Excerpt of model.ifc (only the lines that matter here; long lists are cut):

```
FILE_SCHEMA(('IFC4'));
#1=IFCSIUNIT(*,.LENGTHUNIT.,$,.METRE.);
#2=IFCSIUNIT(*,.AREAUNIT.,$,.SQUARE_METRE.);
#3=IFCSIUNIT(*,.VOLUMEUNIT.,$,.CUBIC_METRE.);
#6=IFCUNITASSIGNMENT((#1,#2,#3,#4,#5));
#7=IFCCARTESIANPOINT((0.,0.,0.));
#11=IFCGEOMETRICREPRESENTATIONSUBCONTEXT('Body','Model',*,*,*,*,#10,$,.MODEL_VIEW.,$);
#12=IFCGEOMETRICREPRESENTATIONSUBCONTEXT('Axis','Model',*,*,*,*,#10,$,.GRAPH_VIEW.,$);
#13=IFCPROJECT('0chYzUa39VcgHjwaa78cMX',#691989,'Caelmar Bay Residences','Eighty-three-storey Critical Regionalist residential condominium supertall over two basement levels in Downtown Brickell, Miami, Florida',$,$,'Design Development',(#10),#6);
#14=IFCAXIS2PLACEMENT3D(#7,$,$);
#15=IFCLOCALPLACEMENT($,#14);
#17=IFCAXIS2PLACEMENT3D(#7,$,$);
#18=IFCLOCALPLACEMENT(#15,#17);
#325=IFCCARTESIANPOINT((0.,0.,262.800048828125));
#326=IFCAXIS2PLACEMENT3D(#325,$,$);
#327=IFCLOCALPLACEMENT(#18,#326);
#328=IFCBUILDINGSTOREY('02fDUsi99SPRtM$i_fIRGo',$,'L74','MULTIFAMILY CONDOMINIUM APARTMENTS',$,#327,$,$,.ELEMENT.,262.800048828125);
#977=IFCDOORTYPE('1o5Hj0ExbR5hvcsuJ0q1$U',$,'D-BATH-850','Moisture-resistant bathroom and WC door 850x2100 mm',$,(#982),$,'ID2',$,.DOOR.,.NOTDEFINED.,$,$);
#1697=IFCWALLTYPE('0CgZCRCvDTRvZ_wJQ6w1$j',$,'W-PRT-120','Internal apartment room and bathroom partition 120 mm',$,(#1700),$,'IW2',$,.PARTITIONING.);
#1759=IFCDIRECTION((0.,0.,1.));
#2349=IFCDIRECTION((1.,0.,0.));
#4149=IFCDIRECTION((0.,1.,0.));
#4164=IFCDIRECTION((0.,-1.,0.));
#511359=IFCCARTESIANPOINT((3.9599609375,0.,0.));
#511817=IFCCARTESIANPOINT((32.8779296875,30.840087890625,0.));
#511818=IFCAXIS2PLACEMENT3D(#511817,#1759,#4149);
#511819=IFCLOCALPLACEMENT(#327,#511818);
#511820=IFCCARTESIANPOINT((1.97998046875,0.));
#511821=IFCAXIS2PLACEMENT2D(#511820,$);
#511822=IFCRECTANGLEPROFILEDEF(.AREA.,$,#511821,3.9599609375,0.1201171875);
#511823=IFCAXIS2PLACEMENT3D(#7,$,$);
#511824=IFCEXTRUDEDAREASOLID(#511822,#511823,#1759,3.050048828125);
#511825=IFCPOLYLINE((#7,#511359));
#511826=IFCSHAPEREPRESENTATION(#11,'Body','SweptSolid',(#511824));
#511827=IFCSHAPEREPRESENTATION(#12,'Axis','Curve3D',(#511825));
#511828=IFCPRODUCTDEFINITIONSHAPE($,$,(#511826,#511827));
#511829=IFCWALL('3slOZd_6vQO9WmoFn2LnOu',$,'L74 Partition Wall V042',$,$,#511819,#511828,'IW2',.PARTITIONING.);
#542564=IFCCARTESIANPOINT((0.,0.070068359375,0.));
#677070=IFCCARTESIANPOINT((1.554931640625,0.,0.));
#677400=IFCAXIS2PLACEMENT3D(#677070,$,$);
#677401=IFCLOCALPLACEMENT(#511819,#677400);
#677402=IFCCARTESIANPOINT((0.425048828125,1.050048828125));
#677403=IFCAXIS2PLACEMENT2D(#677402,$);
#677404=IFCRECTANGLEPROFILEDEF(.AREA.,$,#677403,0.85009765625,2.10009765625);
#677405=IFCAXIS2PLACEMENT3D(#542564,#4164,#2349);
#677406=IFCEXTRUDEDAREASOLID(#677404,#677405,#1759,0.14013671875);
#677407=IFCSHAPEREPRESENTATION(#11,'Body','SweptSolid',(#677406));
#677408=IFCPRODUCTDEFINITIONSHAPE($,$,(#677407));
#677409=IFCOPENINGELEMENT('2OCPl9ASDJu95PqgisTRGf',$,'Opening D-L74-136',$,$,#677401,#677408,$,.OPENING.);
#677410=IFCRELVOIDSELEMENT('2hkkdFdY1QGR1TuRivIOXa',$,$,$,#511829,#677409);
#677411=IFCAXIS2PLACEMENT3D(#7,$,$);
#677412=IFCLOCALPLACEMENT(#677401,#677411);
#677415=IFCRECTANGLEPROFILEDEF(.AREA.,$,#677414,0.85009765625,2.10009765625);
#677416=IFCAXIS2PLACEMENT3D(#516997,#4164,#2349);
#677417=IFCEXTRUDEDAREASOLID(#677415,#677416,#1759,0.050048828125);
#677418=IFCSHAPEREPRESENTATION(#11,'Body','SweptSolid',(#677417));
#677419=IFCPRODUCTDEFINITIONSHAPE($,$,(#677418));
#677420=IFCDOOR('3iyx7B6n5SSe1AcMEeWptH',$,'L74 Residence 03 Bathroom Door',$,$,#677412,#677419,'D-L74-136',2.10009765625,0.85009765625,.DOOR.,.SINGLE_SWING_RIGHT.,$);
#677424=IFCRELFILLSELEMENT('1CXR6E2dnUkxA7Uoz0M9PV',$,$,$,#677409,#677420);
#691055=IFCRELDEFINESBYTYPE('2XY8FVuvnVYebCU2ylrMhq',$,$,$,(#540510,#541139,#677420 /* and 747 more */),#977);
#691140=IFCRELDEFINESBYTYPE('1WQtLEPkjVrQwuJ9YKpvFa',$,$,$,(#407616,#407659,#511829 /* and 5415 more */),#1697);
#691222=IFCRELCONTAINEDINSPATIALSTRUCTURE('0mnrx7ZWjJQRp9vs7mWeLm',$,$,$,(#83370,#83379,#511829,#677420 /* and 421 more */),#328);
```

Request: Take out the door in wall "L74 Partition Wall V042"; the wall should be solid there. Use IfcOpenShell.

```python
import ifcopenshell
import ifcopenshell.api.feature
import ifcopenshell.api.root
import ifcopenshell.geom
import ifcopenshell.util.shape

model = ifcopenshell.open("model.ifc")
settings = ifcopenshell.geom.settings()


def volume(element):
    """Net volume in cubic metres, openings subtracted."""
    shape = ifcopenshell.geom.create_shape(settings, element)
    return ifcopenshell.util.shape.get_volume(shape.geometry)


door = model.by_guid("3iyx7B6n5SSe1AcMEeWptH")
opening = door.FillsVoids[0].RelatingOpeningElement
wall = opening.VoidsElements[0].RelatingBuildingElement
before = volume(wall)

ifcopenshell.api.root.remove_product(model, product=door)
ifcopenshell.api.feature.remove_feature(model, feature=opening)

after = volume(wall)

print(f"wall volume {before:.3f} -> {after:.3f} m3")

model.write("model-out.ifc")
```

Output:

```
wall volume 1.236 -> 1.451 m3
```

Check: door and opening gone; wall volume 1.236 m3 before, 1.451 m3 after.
